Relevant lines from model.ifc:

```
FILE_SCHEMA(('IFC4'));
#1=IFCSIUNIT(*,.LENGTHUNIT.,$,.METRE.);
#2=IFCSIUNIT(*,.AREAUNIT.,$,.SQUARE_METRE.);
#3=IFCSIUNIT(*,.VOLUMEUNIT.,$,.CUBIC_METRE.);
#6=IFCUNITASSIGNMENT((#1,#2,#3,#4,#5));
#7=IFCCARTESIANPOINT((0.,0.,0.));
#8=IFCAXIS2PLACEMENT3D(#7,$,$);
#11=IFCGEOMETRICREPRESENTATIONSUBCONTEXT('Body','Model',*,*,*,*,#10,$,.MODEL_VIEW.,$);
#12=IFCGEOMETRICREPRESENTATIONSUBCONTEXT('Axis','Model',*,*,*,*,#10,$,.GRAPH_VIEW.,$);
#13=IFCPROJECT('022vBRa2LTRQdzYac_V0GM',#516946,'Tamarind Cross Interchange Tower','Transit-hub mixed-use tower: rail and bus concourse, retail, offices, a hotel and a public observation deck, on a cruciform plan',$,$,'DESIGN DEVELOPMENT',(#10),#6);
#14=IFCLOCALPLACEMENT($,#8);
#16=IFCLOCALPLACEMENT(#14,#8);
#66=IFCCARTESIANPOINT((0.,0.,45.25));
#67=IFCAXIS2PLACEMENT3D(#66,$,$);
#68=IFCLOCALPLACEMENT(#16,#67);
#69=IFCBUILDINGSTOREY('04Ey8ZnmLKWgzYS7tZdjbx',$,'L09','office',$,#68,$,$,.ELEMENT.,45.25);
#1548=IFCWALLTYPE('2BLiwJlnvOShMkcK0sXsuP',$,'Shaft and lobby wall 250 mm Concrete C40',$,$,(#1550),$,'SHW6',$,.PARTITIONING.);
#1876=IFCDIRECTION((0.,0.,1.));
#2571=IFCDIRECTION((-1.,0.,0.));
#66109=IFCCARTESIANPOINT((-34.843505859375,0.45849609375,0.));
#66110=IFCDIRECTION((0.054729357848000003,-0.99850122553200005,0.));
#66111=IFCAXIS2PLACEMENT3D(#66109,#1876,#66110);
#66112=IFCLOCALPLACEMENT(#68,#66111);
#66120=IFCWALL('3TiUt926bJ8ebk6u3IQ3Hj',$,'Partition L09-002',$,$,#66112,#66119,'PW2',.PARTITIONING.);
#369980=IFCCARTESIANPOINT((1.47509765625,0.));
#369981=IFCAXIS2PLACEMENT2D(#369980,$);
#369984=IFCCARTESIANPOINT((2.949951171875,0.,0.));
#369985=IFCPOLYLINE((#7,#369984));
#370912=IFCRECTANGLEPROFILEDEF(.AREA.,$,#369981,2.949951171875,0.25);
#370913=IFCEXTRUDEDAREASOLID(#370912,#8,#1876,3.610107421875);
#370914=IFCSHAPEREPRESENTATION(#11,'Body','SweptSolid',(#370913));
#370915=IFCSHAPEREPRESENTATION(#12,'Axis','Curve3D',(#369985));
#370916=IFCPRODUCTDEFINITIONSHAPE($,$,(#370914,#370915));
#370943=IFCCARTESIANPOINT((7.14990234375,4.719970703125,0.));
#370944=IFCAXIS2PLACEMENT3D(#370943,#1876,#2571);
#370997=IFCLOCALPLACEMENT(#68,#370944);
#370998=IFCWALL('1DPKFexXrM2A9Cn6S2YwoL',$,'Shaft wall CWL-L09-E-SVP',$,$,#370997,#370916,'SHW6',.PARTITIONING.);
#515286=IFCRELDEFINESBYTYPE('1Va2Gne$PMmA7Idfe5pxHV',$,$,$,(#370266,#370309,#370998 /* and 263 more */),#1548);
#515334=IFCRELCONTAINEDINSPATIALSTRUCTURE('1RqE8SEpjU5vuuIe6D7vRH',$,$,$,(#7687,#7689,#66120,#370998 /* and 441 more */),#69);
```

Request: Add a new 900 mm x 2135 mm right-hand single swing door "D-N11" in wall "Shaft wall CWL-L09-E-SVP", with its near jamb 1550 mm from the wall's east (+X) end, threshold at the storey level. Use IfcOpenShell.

```python
import numpy as np
import ifcopenshell
import ifcopenshell.api.feature
import ifcopenshell.api.geometry
import ifcopenshell.api.root
import ifcopenshell.api.spatial
import ifcopenshell.geom
import ifcopenshell.util.element
import ifcopenshell.util.placement
import ifcopenshell.util.representation
import ifcopenshell.util.shape
import ifcopenshell.util.unit

model = ifcopenshell.open("model.ifc")
unit_scale = ifcopenshell.util.unit.calculate_unit_scale(model)
settings = ifcopenshell.geom.settings()


def volume(element):
    """Net volume in cubic metres, openings subtracted."""
    shape = ifcopenshell.geom.create_shape(settings, element)
    return ifcopenshell.util.shape.get_volume(shape.geometry)


wall = model.by_id(370998)
storey = ifcopenshell.util.element.get_container(wall, ifc_class="IfcBuildingStorey")
context = ifcopenshell.util.representation.get_context(model, "Model", "Body", "MODEL_VIEW")
before = volume(wall)

width, height, from_end, sill = 0.9, 2.135, 1.55, 0.0  # metres

# The wall runs along its own X axis, and the end named is its -X end.
wall_shape = ifcopenshell.geom.create_shape(settings, wall)
x, y, z = ifcopenshell.util.shape.get_vertices(wall_shape.geometry).T
start = x.min() + from_end
face, thickness = float(y.min()), float(y.max() - y.min())
wall_matrix = ifcopenshell.util.placement.get_local_placement(wall.ObjectPlacement)
level = ifcopenshell.util.placement.get_local_placement(storey.ObjectPlacement)[2, 3]


def in_wall(x, y):
    """Placement at x, y metres in the wall's axes, at sill height."""
    matrix = wall_matrix.copy()
    matrix[:, 3] = wall_matrix @ np.array([x / unit_scale, y / unit_scale, 0.0, 1.0])
    matrix[2, 3] = level + sill / unit_scale
    return matrix


# Opening: a box that overshoots both wall faces by 50 mm.
opening = ifcopenshell.api.root.create_entity(model, ifc_class="IfcOpeningElement", predefined_type="OPENING")
box = ifcopenshell.api.geometry.add_wall_representation(
    model, context=context, length=width, height=height, thickness=thickness + 0.1
)
ifcopenshell.api.geometry.assign_representation(model, product=opening, representation=box)
ifcopenshell.api.geometry.edit_object_placement(model, product=opening, matrix=in_wall(start, face - 0.05), is_si=False)
ifcopenshell.api.feature.add_feature(model, feature=opening, element=wall)

door = ifcopenshell.api.root.create_entity(model, ifc_class="IfcDoor", name="D-N11", predefined_type="DOOR")
door.OverallWidth, door.OverallHeight = width / unit_scale, height / unit_scale
door.OperationType = "SINGLE_SWING_RIGHT"
body = ifcopenshell.api.geometry.add_door_representation(
    model,
    context=context,
    overall_width=door.OverallWidth,
    overall_height=door.OverallHeight,
    operation_type="SINGLE_SWING_RIGHT",
    lining_properties={"LiningDepth": thickness / unit_scale, "ThresholdDepth": thickness / unit_scale},
)
ifcopenshell.api.geometry.assign_representation(model, product=door, representation=body)
ifcopenshell.api.spatial.assign_container(model, products=[door], relating_structure=storey)
ifcopenshell.api.feature.add_filling(model, opening=opening, element=door)

# The lining spans the wall, so the door starts at the wall face.
ifcopenshell.api.geometry.edit_object_placement(model, product=door, matrix=in_wall(start, face), is_si=False)

after = volume(wall)

print(f"wall volume {before:.3f} -> {after:.3f} m3")

model.write("model-out.ifc")
```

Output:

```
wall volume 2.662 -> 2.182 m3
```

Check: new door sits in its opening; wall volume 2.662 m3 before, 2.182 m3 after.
